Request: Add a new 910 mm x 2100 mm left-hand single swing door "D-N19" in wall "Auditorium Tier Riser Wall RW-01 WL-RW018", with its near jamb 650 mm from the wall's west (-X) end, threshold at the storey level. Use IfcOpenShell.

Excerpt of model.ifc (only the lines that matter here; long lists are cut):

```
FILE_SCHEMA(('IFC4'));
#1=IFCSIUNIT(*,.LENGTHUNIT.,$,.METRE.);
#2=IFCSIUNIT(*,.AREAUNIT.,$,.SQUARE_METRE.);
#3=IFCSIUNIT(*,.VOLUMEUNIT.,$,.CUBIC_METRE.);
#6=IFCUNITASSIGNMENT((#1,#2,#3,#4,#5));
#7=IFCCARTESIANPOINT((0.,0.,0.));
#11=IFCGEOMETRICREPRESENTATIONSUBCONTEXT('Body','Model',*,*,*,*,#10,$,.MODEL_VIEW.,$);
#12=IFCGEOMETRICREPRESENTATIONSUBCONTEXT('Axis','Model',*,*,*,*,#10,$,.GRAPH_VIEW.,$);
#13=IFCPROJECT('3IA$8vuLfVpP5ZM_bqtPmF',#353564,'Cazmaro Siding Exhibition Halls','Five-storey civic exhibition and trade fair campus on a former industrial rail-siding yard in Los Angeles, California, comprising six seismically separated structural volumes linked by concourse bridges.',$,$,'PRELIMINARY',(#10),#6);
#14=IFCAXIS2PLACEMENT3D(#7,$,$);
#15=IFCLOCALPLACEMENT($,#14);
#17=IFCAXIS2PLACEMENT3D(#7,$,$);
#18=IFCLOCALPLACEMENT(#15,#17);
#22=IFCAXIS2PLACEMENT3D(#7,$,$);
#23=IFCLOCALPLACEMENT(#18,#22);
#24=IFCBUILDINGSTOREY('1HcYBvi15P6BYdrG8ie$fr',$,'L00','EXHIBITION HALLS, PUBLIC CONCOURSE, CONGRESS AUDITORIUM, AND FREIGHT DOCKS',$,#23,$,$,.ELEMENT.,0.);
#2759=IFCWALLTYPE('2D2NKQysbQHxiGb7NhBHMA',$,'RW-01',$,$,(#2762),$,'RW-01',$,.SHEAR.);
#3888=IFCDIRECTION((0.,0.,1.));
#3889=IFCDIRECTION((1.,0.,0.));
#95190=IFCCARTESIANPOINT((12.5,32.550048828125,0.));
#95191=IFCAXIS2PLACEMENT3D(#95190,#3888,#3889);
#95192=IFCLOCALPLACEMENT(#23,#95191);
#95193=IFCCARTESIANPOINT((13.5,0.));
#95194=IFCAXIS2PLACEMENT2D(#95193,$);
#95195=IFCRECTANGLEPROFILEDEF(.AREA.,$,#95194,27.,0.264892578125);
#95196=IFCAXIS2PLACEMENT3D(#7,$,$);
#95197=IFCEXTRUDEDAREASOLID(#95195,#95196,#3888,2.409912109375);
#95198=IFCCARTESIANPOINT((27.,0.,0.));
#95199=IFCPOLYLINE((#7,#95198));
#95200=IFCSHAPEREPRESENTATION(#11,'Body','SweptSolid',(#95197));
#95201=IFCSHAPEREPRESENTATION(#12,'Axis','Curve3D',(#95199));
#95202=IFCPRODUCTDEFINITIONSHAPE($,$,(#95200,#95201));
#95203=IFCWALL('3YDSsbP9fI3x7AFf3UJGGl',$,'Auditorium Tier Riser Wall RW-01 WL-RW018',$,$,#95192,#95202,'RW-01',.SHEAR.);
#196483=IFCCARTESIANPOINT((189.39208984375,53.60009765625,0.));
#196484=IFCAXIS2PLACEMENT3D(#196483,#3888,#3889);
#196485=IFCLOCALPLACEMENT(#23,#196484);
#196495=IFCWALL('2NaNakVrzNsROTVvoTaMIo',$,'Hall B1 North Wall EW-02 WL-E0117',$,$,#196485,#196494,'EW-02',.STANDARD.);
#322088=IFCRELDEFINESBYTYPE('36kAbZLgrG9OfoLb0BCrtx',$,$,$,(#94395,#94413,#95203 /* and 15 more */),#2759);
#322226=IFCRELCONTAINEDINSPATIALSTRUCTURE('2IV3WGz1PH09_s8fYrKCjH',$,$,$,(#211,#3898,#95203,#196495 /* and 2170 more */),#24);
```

```python
import numpy as np
import ifcopenshell
import ifcopenshell.api.feature
import ifcopenshell.api.geometry
import ifcopenshell.api.root
import ifcopenshell.api.spatial
import ifcopenshell.geom
import ifcopenshell.util.element
import ifcopenshell.util.placement
import ifcopenshell.util.representation
import ifcopenshell.util.shape
import ifcopenshell.util.unit

model = ifcopenshell.open("model.ifc")
unit_scale = ifcopenshell.util.unit.calculate_unit_scale(model)
settings = ifcopenshell.geom.settings()


def volume(element):
    """Net volume in cubic metres, openings subtracted."""
    shape = ifcopenshell.geom.create_shape(settings, element)
    return ifcopenshell.util.shape.get_volume(shape.geometry)


wall = model.by_guid("3YDSsbP9fI3x7AFf3UJGGl")
storey = ifcopenshell.util.element.get_container(wall, ifc_class="IfcBuildingStorey")
context = ifcopenshell.util.representation.get_context(model, "Model", "Body", "MODEL_VIEW")
before = volume(wall)

width, height, from_end, sill = 0.91, 2.1, 0.65, 0.0  # metres

# The wall runs along its own X axis, and the end named is its -X end.
wall_shape = ifcopenshell.geom.create_shape(settings, wall)
x, y, z = ifcopenshell.util.shape.get_vertices(wall_shape.geometry).T
start = x.min() + from_end
face, thickness = float(y.min()), float(y.max() - y.min())
wall_matrix = ifcopenshell.util.placement.get_local_placement(wall.ObjectPlacement)
level = ifcopenshell.util.placement.get_local_placement(storey.ObjectPlacement)[2, 3]


def in_wall(x, y):
    """Placement at x, y metres in the wall's axes, at sill height."""
    matrix = wall_matrix.copy()
    matrix[:, 3] = wall_matrix @ np.array([x / unit_scale, y / unit_scale, 0.0, 1.0])
    matrix[2, 3] = level + sill / unit_scale
    return matrix


# Opening: a box that overshoots both wall faces by 50 mm.
opening = ifcopenshell.api.root.create_entity(model, ifc_class="IfcOpeningElement", predefined_type="OPENING")
box = ifcopenshell.api.geometry.add_wall_representation(
    model, context=context, length=width, height=height, thickness=thickness + 0.1
)
ifcopenshell.api.geometry.assign_representation(model, product=opening, representation=box)
ifcopenshell.api.geometry.edit_object_placement(model, product=opening, matrix=in_wall(start, face - 0.05), is_si=False)
ifcopenshell.api.feature.add_feature(model, feature=opening, element=wall)

door = ifcopenshell.api.root.create_entity(model, ifc_class="IfcDoor", name="D-N19", predefined_type="DOOR")
door.OverallWidth, door.OverallHeight = width / unit_scale, height / unit_scale
door.OperationType = "SINGLE_SWING_LEFT"
body = ifcopenshell.api.geometry.add_door_representation(
    model,
    context=context,
    overall_width=door.OverallWidth,
    overall_height=door.OverallHeight,
    operation_type="SINGLE_SWING_LEFT",
    lining_properties={"LiningDepth": thickness / unit_scale, "ThresholdDepth": thickness / unit_scale},
)
ifcopenshell.api.geometry.assign_representation(model, product=door, representation=body)
ifcopenshell.api.spatial.assign_container(model, products=[door], relating_structure=storey)
ifcopenshell.api.feature.add_filling(model, opening=opening, element=door)

# The lining spans the wall, so the door starts at the wall face.
ifcopenshell.api.geometry.edit_object_placement(model, product=door, matrix=in_wall(start, face), is_si=False)

after = volume(wall)

print(f"wall volume {before:.3f} -> {after:.3f} m3")

model.write("model_edited.ifc")
```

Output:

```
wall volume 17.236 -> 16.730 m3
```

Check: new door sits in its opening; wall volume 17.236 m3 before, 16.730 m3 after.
